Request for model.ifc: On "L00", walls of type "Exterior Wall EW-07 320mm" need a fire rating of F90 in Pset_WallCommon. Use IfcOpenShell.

First a look at what the model holds.

```python
import ifcopenshell
import ifcopenshell.util.element

model = ifcopenshell.open("model.ifc")
print(model.schema)
storey = next(s for s in model.by_type("IfcBuildingStorey") if s.Name == "L00")
walls = [e for e in ifcopenshell.util.element.get_decomposition(storey) if e.is_a("IfcWall")]
seen = {}
for e in walls:
    element_type = ifcopenshell.util.element.get_type(e)
    key = (element_type.Name if element_type != e and element_type else None, ifcopenshell.util.element.get_pset(e, "Pset_WallCommon", "FireRating"))
    seen[key] = seen.get(key, 0) + 1
for (name, value), count in sorted(seen.items(), key=str):
    print(count, "x", name, "|", value)
```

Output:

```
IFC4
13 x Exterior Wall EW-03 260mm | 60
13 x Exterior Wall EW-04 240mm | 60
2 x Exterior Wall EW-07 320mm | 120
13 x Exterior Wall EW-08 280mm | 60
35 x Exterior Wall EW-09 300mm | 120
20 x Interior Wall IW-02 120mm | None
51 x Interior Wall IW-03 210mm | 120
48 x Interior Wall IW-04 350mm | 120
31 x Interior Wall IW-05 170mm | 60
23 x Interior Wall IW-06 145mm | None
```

```python
import ifcopenshell
import ifcopenshell.api.pset
import ifcopenshell.util.element

model = ifcopenshell.open("model.ifc")

storey = next(s for s in model.by_type("IfcBuildingStorey") if s.Name == "L00")
walls = [e for e in ifcopenshell.util.element.get_decomposition(storey) if e.is_a("IfcWall")]

count = 0
for e in walls:
    element_type = ifcopenshell.util.element.get_type(e)
    if element_type in (None, e) or element_type.Name != "Exterior Wall EW-07 320mm":
        continue
    # add_pset returns the element's existing set when there is one.
    pset = ifcopenshell.api.pset.add_pset(model, product=e, name="Pset_WallCommon")
    ifcopenshell.api.pset.edit_pset(model, pset=pset, properties={"FireRating": "F90"})
    count += 1

print(count, "walls updated")

model.write("model_updated.ifc")
```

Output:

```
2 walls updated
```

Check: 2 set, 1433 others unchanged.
